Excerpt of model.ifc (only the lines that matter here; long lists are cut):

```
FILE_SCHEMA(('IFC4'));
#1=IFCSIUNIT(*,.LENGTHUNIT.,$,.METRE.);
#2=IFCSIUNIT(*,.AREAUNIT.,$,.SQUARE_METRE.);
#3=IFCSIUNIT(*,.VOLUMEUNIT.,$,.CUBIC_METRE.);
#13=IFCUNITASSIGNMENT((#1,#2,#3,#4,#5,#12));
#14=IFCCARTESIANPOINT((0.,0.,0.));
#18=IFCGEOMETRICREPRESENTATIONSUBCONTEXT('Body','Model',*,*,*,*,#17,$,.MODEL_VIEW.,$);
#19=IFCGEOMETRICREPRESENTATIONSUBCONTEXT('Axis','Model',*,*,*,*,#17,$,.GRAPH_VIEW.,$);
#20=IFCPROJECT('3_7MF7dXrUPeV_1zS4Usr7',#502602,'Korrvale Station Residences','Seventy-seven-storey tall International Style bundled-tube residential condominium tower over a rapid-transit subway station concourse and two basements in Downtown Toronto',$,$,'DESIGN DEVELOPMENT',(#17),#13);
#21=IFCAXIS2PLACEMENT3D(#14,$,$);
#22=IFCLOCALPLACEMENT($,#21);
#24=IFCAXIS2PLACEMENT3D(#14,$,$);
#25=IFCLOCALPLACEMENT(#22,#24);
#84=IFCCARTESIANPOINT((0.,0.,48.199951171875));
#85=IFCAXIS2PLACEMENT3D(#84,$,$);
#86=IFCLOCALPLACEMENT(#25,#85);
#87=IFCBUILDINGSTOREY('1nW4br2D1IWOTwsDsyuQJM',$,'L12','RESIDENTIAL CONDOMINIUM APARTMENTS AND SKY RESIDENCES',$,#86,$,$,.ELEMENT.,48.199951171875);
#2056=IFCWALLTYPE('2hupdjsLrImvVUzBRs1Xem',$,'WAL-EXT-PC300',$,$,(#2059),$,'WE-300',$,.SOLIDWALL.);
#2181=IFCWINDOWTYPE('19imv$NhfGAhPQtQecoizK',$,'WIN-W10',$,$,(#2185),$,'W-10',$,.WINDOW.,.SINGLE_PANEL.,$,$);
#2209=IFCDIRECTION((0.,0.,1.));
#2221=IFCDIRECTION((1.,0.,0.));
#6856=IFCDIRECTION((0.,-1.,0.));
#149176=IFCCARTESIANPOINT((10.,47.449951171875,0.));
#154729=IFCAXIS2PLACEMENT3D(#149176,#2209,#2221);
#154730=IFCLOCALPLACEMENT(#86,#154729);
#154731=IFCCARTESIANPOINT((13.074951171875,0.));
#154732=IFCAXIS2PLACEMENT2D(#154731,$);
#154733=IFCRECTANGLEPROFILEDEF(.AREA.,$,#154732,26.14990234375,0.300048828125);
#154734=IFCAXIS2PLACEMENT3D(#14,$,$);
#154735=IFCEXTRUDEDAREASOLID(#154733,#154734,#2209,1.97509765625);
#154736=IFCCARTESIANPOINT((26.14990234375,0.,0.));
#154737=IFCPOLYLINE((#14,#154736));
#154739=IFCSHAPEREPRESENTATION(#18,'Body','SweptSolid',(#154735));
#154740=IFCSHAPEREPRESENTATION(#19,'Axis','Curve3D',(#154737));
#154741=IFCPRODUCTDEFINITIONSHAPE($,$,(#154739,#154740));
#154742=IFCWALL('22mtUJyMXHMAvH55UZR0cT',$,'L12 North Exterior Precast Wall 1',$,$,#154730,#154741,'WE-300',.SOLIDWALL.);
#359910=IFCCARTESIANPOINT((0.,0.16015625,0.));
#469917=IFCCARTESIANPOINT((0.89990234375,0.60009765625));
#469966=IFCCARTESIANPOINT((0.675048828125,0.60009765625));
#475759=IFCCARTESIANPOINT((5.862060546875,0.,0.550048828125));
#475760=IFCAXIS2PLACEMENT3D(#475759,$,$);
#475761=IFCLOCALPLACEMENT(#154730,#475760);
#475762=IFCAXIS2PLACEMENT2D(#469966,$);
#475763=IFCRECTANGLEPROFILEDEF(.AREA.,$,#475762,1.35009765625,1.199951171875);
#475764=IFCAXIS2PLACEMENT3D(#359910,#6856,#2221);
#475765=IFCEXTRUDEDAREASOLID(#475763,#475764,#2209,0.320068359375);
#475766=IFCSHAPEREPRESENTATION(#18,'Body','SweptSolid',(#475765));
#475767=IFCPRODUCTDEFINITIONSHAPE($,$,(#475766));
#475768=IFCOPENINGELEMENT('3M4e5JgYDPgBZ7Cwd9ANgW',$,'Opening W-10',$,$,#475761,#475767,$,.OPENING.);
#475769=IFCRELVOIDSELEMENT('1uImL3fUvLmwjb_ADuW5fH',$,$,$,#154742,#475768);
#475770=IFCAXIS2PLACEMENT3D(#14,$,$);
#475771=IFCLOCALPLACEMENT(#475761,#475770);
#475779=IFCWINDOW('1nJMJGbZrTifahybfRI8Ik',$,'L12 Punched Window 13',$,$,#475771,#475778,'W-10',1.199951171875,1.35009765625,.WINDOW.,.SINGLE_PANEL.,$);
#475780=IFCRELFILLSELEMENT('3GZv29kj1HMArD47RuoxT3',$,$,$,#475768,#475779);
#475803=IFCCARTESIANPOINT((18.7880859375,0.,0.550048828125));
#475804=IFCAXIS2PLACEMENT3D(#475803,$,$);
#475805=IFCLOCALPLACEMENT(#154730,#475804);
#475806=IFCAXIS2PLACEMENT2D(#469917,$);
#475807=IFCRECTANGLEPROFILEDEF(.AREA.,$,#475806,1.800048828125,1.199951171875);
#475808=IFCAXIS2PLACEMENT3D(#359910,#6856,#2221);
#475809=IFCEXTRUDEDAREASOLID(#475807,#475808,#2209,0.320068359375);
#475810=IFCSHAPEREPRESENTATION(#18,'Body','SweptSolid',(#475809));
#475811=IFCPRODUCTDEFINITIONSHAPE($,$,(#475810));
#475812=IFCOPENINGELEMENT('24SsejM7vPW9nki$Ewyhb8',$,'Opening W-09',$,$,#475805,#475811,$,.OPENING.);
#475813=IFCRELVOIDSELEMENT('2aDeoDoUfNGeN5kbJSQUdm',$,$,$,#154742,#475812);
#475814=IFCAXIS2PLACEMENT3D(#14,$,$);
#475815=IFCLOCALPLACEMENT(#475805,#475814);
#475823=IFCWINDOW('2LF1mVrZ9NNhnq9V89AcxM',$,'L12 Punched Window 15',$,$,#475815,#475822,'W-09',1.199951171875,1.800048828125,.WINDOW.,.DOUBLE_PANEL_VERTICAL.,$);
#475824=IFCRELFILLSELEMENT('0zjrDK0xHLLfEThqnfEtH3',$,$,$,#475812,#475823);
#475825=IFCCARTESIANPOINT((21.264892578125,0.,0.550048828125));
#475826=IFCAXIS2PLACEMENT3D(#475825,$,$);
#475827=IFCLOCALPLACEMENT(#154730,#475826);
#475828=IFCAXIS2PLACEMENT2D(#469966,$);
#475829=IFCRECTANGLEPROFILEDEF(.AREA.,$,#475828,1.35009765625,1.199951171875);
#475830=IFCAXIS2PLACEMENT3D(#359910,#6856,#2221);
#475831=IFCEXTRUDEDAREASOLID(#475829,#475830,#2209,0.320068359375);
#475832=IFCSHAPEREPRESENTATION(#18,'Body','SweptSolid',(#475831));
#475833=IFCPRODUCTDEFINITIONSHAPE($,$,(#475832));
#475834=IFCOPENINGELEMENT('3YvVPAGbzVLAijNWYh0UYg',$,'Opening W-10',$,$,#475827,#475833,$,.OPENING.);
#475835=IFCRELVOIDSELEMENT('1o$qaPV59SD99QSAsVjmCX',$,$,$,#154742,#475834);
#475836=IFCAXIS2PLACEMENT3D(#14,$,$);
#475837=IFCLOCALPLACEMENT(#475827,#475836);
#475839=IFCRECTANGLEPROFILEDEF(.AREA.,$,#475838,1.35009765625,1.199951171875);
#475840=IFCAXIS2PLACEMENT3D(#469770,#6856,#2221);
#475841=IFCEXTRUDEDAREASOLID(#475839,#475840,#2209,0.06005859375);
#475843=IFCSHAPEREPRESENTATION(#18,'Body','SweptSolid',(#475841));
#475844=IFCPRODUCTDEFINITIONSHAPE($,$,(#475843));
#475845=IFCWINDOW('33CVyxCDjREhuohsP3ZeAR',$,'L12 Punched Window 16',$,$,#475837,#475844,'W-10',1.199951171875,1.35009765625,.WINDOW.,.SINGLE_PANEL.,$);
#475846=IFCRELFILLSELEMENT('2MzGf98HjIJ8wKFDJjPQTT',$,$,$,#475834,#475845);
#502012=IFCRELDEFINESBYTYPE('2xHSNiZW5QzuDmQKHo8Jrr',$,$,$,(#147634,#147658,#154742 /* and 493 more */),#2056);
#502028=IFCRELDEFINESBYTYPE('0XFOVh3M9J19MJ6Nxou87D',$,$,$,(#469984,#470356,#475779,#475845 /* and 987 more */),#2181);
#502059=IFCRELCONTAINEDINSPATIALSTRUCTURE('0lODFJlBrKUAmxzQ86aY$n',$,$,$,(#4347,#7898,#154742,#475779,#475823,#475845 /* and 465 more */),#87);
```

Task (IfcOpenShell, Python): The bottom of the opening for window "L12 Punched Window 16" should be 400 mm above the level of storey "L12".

```python
import numpy as np
import ifcopenshell
import ifcopenshell.api.geometry
import ifcopenshell.geom
import ifcopenshell.util.element
import ifcopenshell.util.placement
import ifcopenshell.util.shape
import ifcopenshell.util.unit

model = ifcopenshell.open("model.ifc")
unit_scale = ifcopenshell.util.unit.calculate_unit_scale(model)

window = model.by_guid("33CVyxCDjREhuohsP3ZeAR")
opening = window.FillsVoids[0].RelatingOpeningElement
storey = ifcopenshell.util.element.get_container(window, ifc_class="IfcBuildingStorey")
level = ifcopenshell.util.placement.get_local_placement(storey.ObjectPlacement)[2, 3]

# The opening's origin need not be at the sill, so measure its lowest point.
shape = ifcopenshell.geom.create_shape(ifcopenshell.geom.settings(), opening)
bottom = ifcopenshell.util.shape.get_shape_bottom_elevation(shape, shape.geometry) / unit_scale
dz = level + 0.4 / unit_scale - bottom

shift = np.array([0.0, 0.0, dz])
# The window is placed relative to its opening, so it follows when the opening moves.
matrix = ifcopenshell.util.placement.get_local_placement(opening.ObjectPlacement)
matrix[:3, 3] += shift
ifcopenshell.api.geometry.edit_object_placement(
    model, product=opening, matrix=matrix, is_si=False, should_transform_children=True
)

print(f"moved by {dz * unit_scale:+.3f} m")

model.write("model_edited.ifc")
```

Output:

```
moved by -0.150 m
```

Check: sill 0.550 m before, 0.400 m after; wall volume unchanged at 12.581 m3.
